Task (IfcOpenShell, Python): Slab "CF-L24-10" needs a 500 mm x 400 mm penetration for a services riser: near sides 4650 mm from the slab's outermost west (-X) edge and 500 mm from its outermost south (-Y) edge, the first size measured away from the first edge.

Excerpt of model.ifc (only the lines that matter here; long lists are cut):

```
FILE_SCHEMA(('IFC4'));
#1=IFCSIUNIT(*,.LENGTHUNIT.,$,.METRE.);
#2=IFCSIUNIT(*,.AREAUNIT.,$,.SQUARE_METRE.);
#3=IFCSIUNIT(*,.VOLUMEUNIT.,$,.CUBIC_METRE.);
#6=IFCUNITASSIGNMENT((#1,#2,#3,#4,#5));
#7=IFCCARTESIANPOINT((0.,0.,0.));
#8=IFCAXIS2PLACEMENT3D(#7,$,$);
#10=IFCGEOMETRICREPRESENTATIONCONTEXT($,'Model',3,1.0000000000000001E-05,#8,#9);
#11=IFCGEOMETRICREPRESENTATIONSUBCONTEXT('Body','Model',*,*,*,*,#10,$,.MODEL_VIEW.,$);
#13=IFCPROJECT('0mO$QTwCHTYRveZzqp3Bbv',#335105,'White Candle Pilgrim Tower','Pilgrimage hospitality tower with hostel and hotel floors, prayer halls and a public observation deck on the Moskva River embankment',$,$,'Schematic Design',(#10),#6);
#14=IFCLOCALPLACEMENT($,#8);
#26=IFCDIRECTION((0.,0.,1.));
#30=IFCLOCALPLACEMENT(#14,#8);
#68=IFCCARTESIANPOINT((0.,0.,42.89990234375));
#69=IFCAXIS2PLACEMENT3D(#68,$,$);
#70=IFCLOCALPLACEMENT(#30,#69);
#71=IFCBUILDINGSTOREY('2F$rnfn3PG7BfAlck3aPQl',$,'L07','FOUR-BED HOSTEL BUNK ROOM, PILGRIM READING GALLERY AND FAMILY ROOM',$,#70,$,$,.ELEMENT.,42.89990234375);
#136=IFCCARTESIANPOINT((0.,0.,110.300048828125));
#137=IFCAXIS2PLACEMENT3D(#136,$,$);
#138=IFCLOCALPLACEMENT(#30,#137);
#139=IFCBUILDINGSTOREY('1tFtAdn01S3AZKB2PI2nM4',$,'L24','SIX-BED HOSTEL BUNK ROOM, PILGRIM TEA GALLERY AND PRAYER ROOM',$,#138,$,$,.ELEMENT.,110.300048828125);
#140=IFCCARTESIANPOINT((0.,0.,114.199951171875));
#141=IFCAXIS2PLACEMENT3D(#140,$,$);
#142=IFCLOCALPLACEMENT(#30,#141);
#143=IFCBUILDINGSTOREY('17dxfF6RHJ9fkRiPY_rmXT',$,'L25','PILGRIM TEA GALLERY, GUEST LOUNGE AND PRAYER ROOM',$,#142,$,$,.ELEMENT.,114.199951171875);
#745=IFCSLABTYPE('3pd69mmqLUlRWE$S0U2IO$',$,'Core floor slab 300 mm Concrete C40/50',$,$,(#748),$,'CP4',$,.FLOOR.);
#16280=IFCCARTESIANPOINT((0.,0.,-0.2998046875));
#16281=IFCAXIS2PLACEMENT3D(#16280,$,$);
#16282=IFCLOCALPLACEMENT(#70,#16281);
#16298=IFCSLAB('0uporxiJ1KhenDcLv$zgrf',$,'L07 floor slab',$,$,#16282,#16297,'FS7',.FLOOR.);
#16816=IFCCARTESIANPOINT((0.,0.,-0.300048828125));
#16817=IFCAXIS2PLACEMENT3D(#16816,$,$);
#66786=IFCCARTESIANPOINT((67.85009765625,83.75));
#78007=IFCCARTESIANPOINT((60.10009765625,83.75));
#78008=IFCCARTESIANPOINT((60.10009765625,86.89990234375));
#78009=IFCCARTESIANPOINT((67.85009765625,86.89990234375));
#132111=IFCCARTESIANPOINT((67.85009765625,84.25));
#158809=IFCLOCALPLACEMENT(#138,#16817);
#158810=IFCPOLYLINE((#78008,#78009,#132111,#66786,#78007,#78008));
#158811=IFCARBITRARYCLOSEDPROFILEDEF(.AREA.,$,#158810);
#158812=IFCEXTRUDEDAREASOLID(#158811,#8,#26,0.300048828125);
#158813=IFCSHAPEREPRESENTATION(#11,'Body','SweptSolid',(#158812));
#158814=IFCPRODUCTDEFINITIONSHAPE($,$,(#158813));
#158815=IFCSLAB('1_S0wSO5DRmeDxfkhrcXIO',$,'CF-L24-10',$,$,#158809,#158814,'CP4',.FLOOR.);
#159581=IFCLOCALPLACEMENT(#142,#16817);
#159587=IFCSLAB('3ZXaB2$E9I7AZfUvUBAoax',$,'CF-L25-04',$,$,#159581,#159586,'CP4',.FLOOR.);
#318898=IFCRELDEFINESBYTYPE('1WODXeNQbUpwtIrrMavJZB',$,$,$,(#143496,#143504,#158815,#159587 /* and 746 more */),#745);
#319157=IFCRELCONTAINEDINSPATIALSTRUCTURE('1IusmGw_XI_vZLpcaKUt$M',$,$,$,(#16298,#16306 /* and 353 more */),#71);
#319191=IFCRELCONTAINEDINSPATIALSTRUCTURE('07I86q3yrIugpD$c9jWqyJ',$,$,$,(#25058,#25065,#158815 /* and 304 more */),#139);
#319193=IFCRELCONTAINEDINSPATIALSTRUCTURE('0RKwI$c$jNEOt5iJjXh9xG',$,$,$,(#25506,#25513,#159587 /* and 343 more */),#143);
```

```python
import numpy as np
import ifcopenshell
import ifcopenshell.api.feature
import ifcopenshell.api.geometry
import ifcopenshell.api.root
import ifcopenshell.geom
import ifcopenshell.util.placement
import ifcopenshell.util.representation
import ifcopenshell.util.shape
import ifcopenshell.util.unit

model = ifcopenshell.open("model.ifc")
unit_scale = ifcopenshell.util.unit.calculate_unit_scale(model)
settings = ifcopenshell.geom.settings()


def volume(element):
    """Net volume in cubic metres, openings subtracted."""
    shape = ifcopenshell.geom.create_shape(settings, element)
    return ifcopenshell.util.shape.get_volume(shape.geometry)


slab = model.by_id(158815)
before = volume(slab)

# Extent in the slab's own axes, in metres. The edges named are its -X and -Y sides.
slab_shape = ifcopenshell.geom.create_shape(settings, slab)
vertices = ifcopenshell.util.shape.get_vertices(slab_shape.geometry)
x_min, y_min, bottom = vertices.min(axis=0)
top = vertices[:, 2].max()

opening = ifcopenshell.api.root.create_entity(model, ifc_class="IfcOpeningElement", name="Services riser opening", predefined_type="OPENING")
context = ifcopenshell.util.representation.get_context(model, "Model", "Body", "MODEL_VIEW")
width, depth = 0.5, 0.4
outline = [(0.0, 0.0), (width, 0.0), (width, depth), (0.0, depth), (0.0, 0.0)]
# Overshoot both faces by 50 mm so the cut is clean.
shape = ifcopenshell.api.geometry.add_slab_representation(
    model, context=context, depth=top - bottom + 0.1, polyline=outline
)
ifcopenshell.api.geometry.assign_representation(model, product=opening, representation=shape)

matrix = ifcopenshell.util.placement.get_local_placement(slab.ObjectPlacement)
matrix[:, 3] = matrix @ np.append(np.array([x_min + 4.65, y_min + 0.5, bottom - 0.05]) / unit_scale, 1.0)
ifcopenshell.api.geometry.edit_object_placement(model, product=opening, matrix=matrix, is_si=False)
ifcopenshell.api.feature.add_feature(model, feature=opening, element=slab)

after = volume(slab)

print(f"slab volume {before:.3f} -> {after:.3f} m3")

model.write("model-out.ifc")
```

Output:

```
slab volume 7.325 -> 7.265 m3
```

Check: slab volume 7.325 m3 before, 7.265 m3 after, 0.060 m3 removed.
